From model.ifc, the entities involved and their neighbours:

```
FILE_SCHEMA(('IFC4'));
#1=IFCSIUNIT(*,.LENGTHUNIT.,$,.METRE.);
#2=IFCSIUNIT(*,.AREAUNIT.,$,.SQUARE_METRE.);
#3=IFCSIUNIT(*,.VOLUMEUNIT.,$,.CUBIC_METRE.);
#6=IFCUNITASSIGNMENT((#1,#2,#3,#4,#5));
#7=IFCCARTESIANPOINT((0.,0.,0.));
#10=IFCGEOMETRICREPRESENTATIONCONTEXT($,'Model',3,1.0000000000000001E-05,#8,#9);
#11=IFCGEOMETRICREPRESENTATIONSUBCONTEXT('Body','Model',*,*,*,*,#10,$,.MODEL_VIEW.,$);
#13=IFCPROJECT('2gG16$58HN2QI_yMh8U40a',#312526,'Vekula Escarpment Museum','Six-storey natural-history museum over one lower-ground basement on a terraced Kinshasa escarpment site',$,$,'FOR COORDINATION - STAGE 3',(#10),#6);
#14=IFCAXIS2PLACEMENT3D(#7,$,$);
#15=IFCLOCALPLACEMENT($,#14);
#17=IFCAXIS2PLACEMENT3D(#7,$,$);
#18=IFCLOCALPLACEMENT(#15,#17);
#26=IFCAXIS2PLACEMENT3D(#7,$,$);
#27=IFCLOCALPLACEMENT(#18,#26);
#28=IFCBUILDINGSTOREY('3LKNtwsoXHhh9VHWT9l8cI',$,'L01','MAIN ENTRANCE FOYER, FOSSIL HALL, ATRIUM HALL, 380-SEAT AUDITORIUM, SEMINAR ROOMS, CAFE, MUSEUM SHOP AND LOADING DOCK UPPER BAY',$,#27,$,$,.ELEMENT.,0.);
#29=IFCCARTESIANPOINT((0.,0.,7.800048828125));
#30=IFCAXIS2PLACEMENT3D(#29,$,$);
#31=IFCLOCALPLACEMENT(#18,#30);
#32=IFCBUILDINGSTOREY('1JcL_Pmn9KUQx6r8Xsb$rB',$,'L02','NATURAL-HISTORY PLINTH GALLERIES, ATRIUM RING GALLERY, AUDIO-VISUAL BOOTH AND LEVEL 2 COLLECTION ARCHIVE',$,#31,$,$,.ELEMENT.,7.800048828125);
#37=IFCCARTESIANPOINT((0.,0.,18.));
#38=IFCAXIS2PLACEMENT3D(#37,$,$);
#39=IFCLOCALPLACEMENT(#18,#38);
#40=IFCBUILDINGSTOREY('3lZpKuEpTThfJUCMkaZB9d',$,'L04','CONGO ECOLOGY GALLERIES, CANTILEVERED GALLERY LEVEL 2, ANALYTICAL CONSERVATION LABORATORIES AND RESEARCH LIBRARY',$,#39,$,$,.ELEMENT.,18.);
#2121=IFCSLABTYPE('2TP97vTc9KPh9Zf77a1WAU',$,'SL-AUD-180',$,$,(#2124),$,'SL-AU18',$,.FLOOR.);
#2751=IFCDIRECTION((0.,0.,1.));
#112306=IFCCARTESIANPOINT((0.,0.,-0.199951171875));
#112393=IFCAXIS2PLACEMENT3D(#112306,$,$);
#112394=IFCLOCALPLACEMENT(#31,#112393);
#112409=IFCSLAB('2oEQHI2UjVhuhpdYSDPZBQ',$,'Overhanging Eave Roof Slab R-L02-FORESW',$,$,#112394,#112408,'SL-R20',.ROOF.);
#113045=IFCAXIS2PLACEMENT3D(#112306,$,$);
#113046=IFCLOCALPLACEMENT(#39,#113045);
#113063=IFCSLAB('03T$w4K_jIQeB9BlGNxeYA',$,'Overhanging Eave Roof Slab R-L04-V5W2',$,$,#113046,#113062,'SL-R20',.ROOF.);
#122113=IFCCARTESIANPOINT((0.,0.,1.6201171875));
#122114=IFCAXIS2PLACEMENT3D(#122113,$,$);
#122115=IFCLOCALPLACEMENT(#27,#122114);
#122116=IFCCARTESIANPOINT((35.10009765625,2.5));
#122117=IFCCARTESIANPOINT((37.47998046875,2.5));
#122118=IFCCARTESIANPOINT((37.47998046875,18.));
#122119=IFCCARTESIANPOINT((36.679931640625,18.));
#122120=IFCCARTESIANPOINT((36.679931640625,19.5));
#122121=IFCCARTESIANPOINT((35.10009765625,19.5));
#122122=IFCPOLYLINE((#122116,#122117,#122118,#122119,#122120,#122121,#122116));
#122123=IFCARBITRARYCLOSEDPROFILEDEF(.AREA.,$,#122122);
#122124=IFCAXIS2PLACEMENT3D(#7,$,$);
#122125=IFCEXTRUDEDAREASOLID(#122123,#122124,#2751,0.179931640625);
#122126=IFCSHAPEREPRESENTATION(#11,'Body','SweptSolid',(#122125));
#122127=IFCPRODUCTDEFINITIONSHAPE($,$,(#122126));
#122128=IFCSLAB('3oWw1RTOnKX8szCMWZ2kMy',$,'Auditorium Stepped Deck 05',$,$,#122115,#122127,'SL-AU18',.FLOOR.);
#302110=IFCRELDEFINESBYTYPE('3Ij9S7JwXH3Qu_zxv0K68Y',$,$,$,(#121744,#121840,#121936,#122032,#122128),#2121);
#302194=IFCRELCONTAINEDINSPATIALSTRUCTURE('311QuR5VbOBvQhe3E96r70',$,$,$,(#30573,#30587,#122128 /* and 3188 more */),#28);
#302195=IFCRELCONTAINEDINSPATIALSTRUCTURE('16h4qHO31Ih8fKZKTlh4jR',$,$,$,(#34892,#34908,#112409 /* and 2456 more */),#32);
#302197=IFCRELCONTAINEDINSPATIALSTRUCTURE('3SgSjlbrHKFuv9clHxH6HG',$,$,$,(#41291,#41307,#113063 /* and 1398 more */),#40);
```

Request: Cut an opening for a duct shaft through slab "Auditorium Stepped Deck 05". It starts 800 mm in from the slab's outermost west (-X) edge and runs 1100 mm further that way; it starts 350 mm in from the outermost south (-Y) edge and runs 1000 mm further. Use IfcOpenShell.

```python
import numpy as np
import ifcopenshell
import ifcopenshell.api.feature
import ifcopenshell.api.geometry
import ifcopenshell.api.root
import ifcopenshell.geom
import ifcopenshell.util.placement
import ifcopenshell.util.representation
import ifcopenshell.util.shape
import ifcopenshell.util.unit

model = ifcopenshell.open("model.ifc")
unit_scale = ifcopenshell.util.unit.calculate_unit_scale(model)
settings = ifcopenshell.geom.settings()


def volume(element):
    """Net volume in cubic metres, openings subtracted."""
    shape = ifcopenshell.geom.create_shape(settings, element)
    return ifcopenshell.util.shape.get_volume(shape.geometry)


slab = model.by_guid("3oWw1RTOnKX8szCMWZ2kMy")
before = volume(slab)

# Extent in the slab's own axes, in metres. The edges named are its -X and -Y sides.
slab_shape = ifcopenshell.geom.create_shape(settings, slab)
vertices = ifcopenshell.util.shape.get_vertices(slab_shape.geometry)
x_min, y_min, bottom = vertices.min(axis=0)
top = vertices[:, 2].max()

opening = ifcopenshell.api.root.create_entity(model, ifc_class="IfcOpeningElement", name="Duct shaft opening", predefined_type="OPENING")
context = ifcopenshell.util.representation.get_context(model, "Model", "Body", "MODEL_VIEW")
width, depth = 1.1, 1
outline = [(0.0, 0.0), (width, 0.0), (width, depth), (0.0, depth), (0.0, 0.0)]
# Overshoot both faces by 50 mm so the cut is clean.
shape = ifcopenshell.api.geometry.add_slab_representation(
    model, context=context, depth=top - bottom + 0.1, polyline=outline
)
ifcopenshell.api.geometry.assign_representation(model, product=opening, representation=shape)

matrix = ifcopenshell.util.placement.get_local_placement(slab.ObjectPlacement)
matrix[:, 3] = matrix @ np.append(np.array([x_min + 0.8, y_min + 0.35, bottom - 0.05]) / unit_scale, 1.0)
ifcopenshell.api.geometry.edit_object_placement(model, product=opening, matrix=matrix, is_si=False)
ifcopenshell.api.feature.add_feature(model, feature=opening, element=slab)

after = volume(slab)

print(f"slab volume {before:.3f} -> {after:.3f} m3")

model.write("model_edited.ifc")
```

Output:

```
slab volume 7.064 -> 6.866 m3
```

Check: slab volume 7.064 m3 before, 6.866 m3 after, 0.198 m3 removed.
